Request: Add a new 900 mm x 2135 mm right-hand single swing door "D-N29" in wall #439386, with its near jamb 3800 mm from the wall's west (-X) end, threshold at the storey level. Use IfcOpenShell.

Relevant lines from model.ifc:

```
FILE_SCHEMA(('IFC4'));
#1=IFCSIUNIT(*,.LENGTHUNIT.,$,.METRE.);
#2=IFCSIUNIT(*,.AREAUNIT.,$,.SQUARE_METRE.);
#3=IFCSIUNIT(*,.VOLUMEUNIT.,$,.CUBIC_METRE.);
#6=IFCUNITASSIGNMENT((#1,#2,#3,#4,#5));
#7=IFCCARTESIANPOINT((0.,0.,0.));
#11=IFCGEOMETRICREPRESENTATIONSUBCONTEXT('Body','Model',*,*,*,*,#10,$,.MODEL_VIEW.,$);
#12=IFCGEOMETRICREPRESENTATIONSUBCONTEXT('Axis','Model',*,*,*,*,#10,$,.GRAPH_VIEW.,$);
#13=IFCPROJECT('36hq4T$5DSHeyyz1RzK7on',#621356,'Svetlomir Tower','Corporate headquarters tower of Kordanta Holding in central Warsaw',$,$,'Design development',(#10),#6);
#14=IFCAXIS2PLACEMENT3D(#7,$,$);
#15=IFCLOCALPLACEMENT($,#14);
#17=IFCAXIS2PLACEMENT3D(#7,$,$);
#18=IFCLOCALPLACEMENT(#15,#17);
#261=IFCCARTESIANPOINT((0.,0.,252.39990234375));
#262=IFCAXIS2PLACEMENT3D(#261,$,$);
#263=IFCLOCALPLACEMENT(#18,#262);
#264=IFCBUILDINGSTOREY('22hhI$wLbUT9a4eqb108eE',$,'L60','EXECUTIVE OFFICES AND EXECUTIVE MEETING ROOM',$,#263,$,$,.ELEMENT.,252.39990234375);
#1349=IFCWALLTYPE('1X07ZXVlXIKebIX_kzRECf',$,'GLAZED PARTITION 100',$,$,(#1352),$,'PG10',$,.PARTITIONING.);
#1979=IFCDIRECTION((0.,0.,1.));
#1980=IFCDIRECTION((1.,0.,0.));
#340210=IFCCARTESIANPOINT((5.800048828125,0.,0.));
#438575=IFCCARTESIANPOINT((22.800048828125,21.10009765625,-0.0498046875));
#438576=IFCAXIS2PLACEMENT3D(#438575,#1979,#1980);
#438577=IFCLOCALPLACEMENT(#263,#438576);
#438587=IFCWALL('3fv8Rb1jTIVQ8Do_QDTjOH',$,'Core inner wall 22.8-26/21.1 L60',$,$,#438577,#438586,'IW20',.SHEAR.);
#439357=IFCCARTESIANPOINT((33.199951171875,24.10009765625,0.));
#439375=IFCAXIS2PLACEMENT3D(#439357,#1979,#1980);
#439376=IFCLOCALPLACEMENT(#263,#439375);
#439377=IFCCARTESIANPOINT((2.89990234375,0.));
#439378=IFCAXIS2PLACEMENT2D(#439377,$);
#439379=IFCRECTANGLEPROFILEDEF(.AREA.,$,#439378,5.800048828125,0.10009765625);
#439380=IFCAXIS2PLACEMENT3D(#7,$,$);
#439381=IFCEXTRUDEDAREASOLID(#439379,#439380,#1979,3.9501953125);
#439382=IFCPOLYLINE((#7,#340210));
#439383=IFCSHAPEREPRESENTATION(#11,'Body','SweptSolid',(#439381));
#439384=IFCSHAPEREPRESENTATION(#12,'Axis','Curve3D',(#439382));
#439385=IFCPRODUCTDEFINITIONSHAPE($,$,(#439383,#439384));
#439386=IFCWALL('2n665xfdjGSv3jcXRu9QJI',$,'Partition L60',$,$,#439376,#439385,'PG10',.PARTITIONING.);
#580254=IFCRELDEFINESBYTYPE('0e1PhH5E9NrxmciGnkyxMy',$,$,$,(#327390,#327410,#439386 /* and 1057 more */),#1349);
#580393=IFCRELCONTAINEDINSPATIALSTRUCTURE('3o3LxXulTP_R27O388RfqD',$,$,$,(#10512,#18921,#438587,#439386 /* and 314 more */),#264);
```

```python
import numpy as np
import ifcopenshell
import ifcopenshell.api.feature
import ifcopenshell.api.geometry
import ifcopenshell.api.root
import ifcopenshell.api.spatial
import ifcopenshell.geom
import ifcopenshell.util.element
import ifcopenshell.util.placement
import ifcopenshell.util.representation
import ifcopenshell.util.shape
import ifcopenshell.util.unit

model = ifcopenshell.open("model.ifc")
unit_scale = ifcopenshell.util.unit.calculate_unit_scale(model)
settings = ifcopenshell.geom.settings()


def volume(element):
    """Net volume in cubic metres, openings subtracted."""
    shape = ifcopenshell.geom.create_shape(settings, element)
    return ifcopenshell.util.shape.get_volume(shape.geometry)


wall = model.by_guid("2n665xfdjGSv3jcXRu9QJI")
storey = ifcopenshell.util.element.get_container(wall, ifc_class="IfcBuildingStorey")
context = ifcopenshell.util.representation.get_context(model, "Model", "Body", "MODEL_VIEW")
before = volume(wall)

width, height, from_end, sill = 0.9, 2.135, 3.8, 0.0  # metres

# The wall runs along its own X axis, and the end named is its -X end.
wall_shape = ifcopenshell.geom.create_shape(settings, wall)
x, y, z = ifcopenshell.util.shape.get_vertices(wall_shape.geometry).T
start = x.min() + from_end
face, thickness = float(y.min()), float(y.max() - y.min())
wall_matrix = ifcopenshell.util.placement.get_local_placement(wall.ObjectPlacement)
level = ifcopenshell.util.placement.get_local_placement(storey.ObjectPlacement)[2, 3]


def in_wall(x, y):
    """Placement at x, y metres in the wall's axes, at sill height."""
    matrix = wall_matrix.copy()
    matrix[:, 3] = wall_matrix @ np.array([x / unit_scale, y / unit_scale, 0.0, 1.0])
    matrix[2, 3] = level + sill / unit_scale
    return matrix


# Opening: a box that overshoots both wall faces by 50 mm.
opening = ifcopenshell.api.root.create_entity(model, ifc_class="IfcOpeningElement", predefined_type="OPENING")
box = ifcopenshell.api.geometry.add_wall_representation(
    model, context=context, length=width, height=height, thickness=thickness + 0.1
)
ifcopenshell.api.geometry.assign_representation(model, product=opening, representation=box)
ifcopenshell.api.geometry.edit_object_placement(model, product=opening, matrix=in_wall(start, face - 0.05), is_si=False)
ifcopenshell.api.feature.add_feature(model, feature=opening, element=wall)

door = ifcopenshell.api.root.create_entity(model, ifc_class="IfcDoor", name="D-N29", predefined_type="DOOR")
door.OverallWidth, door.OverallHeight = width / unit_scale, height / unit_scale
door.OperationType = "SINGLE_SWING_RIGHT"
body = ifcopenshell.api.geometry.add_door_representation(
    model,
    context=context,
    overall_width=door.OverallWidth,
    overall_height=door.OverallHeight,
    operation_type="SINGLE_SWING_RIGHT",
    lining_properties={"LiningDepth": thickness / unit_scale, "ThresholdDepth": thickness / unit_scale},
)
ifcopenshell.api.geometry.assign_representation(model, product=door, representation=body)
ifcopenshell.api.spatial.assign_container(model, products=[door], relating_structure=storey)
ifcopenshell.api.feature.add_filling(model, opening=opening, element=door)

# The lining spans the wall, so the door starts at the wall face.
ifcopenshell.api.geometry.edit_object_placement(model, product=door, matrix=in_wall(start, face), is_si=False)

after = volume(wall)

print(f"wall volume {before:.3f} -> {after:.3f} m3")

model.write("model_edited.ifc")
```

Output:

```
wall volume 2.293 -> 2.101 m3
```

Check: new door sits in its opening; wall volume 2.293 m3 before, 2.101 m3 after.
